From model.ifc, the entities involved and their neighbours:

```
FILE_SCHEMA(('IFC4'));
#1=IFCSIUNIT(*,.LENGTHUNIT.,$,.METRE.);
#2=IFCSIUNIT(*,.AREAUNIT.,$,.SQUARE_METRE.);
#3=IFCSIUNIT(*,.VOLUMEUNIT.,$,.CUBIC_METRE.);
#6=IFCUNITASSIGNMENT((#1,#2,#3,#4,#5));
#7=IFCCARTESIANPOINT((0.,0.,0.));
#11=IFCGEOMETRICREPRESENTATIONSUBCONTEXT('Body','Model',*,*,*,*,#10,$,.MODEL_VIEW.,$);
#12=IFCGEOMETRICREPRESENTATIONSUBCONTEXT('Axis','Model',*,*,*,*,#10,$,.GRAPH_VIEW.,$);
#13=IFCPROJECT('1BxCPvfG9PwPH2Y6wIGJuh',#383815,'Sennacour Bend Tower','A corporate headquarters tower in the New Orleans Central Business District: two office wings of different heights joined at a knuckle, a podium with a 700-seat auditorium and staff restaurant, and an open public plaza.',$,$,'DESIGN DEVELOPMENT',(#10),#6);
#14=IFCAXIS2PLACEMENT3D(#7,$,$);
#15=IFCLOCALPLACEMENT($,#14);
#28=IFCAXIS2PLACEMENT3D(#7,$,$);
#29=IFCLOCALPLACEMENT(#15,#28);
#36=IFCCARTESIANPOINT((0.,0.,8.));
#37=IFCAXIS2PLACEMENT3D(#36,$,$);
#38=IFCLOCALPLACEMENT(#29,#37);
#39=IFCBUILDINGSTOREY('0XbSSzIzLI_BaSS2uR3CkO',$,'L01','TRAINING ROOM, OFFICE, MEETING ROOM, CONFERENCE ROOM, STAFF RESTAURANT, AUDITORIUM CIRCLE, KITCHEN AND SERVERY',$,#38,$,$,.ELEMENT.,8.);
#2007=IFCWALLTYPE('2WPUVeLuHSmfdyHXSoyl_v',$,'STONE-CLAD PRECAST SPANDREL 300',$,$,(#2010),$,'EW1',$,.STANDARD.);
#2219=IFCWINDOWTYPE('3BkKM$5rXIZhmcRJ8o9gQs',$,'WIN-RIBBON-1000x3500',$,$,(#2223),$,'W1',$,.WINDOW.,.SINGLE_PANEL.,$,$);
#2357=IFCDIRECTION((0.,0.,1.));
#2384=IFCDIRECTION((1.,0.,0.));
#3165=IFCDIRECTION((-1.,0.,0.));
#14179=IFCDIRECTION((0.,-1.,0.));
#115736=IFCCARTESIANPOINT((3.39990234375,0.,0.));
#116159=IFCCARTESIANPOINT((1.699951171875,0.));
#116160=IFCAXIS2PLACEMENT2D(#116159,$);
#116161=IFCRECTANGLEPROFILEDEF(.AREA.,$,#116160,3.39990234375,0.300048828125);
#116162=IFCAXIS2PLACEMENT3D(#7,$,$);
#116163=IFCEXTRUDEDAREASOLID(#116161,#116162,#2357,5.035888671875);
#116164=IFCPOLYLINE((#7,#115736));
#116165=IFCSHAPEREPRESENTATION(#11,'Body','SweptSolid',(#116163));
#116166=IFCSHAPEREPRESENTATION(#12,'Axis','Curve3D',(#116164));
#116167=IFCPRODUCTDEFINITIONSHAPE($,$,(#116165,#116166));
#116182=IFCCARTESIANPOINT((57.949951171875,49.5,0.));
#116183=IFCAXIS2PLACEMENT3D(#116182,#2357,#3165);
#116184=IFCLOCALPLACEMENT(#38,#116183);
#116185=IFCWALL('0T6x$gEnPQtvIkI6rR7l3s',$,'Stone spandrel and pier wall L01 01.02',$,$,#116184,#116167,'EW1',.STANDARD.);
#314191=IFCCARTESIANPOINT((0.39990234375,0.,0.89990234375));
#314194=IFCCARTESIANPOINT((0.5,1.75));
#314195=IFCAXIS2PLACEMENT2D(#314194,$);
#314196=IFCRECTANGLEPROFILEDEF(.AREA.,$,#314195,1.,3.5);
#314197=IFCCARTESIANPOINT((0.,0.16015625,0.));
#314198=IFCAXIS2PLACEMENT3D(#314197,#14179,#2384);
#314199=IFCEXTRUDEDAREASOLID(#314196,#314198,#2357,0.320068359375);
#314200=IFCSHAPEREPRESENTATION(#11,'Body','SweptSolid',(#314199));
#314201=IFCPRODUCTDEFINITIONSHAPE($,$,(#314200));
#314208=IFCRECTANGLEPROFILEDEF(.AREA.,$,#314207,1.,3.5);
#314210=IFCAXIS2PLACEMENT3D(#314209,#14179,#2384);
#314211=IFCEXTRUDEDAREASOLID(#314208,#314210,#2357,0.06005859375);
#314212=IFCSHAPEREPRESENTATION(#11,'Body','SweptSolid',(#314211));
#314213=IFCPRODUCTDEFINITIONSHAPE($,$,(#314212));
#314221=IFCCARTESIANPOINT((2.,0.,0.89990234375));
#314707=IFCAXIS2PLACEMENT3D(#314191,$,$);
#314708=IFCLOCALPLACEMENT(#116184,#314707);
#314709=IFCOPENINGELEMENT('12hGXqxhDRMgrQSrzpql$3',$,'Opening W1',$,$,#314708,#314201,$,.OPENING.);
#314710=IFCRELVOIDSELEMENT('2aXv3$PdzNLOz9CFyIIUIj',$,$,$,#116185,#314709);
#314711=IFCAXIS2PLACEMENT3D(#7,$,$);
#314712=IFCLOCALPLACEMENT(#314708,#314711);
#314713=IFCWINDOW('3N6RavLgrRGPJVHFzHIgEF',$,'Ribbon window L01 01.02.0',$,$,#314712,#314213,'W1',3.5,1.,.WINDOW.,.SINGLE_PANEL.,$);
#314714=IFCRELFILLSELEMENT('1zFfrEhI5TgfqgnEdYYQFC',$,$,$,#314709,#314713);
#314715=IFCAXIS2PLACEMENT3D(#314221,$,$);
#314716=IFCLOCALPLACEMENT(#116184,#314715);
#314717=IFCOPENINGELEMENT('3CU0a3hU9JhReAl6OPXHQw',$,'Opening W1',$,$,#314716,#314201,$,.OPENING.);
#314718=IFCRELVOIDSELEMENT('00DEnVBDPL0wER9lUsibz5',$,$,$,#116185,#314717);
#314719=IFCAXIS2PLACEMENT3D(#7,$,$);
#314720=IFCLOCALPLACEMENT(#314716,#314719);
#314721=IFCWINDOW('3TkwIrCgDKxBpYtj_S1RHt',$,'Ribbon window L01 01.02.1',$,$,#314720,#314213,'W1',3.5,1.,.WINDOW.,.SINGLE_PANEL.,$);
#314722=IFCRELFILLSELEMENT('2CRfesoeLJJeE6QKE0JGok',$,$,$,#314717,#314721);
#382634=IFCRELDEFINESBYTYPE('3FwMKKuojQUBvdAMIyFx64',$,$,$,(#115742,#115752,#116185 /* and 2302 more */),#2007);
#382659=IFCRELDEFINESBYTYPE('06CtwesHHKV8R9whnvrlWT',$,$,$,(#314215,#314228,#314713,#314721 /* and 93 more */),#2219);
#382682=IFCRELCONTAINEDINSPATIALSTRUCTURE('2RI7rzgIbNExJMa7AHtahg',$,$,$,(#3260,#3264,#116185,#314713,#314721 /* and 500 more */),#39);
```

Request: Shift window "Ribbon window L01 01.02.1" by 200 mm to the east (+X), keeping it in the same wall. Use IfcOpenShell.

```python
import ifcopenshell
import ifcopenshell.api.geometry
import ifcopenshell.util.placement
import ifcopenshell.util.unit

model = ifcopenshell.open("model.ifc")
unit_scale = ifcopenshell.util.unit.calculate_unit_scale(model)

window = model.by_guid("3TkwIrCgDKxBpYtj_S1RHt")
opening = window.FillsVoids[0].RelatingOpeningElement
wall = opening.VoidsElements[0].RelatingBuildingElement

wall_matrix = ifcopenshell.util.placement.get_local_placement(wall.ObjectPlacement)
shift = wall_matrix[:3, 0] * -0.2 / unit_scale
before = ifcopenshell.util.placement.get_local_placement(window.ObjectPlacement)[:3, 3].copy()

# The window is placed relative to its opening, so it follows when the opening moves.
matrix = ifcopenshell.util.placement.get_local_placement(opening.ObjectPlacement)
matrix[:3, 3] += shift
ifcopenshell.api.geometry.edit_object_placement(
    model, product=opening, matrix=matrix, is_si=False, should_transform_children=True
)

after = ifcopenshell.util.placement.get_local_placement(window.ObjectPlacement)[:3, 3]
print("window moved by", (after - before).round(3) + 0.0)

model.write("model_updated.ifc")
```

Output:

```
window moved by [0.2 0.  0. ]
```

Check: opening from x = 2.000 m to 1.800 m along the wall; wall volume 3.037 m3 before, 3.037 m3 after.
